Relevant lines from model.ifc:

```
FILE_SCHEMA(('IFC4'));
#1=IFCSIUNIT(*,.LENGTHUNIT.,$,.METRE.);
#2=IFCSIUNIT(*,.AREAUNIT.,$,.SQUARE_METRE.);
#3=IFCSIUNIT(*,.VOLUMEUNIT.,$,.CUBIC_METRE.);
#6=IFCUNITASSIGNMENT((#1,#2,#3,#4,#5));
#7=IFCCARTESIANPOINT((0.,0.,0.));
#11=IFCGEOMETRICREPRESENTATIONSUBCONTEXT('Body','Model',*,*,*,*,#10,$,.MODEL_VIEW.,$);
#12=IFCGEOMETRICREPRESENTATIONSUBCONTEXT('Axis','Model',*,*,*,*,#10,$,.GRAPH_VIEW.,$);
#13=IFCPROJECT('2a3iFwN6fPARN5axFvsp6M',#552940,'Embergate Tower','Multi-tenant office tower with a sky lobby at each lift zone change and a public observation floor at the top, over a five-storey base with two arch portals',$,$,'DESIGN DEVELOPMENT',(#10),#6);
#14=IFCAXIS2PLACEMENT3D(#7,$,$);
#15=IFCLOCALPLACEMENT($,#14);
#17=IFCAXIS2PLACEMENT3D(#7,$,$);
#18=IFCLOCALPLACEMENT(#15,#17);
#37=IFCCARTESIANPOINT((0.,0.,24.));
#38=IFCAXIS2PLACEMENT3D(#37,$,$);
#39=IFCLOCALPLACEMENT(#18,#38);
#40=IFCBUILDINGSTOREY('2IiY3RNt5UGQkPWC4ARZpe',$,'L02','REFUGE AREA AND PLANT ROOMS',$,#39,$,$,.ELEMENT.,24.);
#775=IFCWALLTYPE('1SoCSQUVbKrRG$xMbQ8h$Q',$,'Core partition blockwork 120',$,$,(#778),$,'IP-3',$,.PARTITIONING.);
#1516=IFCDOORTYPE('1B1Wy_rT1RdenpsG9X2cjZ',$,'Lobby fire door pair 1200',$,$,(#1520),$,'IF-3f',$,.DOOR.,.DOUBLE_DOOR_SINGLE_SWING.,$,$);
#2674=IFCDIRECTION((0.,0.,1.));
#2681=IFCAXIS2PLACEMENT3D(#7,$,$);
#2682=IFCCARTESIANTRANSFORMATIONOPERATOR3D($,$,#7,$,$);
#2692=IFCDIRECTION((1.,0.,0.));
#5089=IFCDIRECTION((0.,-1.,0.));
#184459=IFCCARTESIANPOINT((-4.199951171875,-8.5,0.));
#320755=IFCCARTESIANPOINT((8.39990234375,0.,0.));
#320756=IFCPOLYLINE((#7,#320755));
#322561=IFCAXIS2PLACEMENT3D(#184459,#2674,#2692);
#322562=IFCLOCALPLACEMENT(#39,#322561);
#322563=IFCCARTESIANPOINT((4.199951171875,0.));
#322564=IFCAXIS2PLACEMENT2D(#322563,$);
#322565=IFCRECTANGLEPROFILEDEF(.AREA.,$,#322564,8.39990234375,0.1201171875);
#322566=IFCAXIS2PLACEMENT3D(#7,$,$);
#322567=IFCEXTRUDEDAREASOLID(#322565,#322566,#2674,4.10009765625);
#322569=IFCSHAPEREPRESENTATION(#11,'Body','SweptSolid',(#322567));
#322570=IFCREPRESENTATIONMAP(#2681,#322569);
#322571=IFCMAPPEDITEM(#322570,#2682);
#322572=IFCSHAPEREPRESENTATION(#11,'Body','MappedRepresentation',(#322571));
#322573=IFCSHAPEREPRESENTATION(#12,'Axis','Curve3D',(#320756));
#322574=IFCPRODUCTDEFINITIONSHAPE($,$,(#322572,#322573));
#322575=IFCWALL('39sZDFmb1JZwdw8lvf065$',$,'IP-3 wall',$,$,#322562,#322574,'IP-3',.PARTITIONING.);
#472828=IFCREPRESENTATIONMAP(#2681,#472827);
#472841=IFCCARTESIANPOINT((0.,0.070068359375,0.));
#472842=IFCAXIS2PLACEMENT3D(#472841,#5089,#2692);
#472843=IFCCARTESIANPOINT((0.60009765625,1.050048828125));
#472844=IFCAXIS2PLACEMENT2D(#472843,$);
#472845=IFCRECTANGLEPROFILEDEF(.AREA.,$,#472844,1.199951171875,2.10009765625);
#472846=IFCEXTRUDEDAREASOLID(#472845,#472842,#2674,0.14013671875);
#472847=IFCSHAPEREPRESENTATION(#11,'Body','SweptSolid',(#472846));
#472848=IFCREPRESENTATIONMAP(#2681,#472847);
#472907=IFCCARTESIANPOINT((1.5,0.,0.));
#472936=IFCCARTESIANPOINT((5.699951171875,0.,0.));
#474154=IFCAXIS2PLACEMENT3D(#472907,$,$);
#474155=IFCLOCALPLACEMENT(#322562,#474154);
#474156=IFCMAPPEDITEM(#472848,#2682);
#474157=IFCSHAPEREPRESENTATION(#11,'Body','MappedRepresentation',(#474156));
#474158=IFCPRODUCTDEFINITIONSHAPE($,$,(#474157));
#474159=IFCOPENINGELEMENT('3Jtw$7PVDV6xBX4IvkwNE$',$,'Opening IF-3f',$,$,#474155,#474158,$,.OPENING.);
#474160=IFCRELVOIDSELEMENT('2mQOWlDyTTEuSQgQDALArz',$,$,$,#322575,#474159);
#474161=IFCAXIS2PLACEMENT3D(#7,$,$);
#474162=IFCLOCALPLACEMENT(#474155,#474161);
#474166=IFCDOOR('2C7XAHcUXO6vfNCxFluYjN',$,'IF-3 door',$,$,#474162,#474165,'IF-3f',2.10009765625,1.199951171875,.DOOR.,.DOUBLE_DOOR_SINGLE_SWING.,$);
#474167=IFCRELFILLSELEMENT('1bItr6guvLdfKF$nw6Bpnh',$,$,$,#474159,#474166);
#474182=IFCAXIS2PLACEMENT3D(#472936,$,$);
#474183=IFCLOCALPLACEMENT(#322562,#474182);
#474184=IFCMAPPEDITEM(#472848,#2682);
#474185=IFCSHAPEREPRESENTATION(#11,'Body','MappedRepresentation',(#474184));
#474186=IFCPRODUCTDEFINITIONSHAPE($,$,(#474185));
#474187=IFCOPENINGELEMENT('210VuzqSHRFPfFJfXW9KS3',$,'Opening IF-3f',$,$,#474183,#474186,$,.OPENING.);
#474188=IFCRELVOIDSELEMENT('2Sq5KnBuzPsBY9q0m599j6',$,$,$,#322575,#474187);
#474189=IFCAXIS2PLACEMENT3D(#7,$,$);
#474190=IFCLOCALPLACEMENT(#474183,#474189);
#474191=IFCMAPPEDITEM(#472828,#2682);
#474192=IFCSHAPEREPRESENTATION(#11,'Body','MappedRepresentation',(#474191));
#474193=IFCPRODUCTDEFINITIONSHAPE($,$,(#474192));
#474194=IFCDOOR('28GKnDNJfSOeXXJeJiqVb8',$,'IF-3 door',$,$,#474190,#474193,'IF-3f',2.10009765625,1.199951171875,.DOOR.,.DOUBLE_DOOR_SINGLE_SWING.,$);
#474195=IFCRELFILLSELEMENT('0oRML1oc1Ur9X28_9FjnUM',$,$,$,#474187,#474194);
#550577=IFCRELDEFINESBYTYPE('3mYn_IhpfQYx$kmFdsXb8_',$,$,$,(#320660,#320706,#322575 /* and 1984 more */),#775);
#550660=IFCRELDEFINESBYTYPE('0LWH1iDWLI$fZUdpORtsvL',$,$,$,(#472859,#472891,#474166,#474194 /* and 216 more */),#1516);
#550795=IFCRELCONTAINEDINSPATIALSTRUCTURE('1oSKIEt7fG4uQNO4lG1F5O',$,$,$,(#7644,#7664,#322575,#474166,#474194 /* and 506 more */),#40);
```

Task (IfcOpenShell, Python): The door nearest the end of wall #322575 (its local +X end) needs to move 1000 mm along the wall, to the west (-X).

```python
import ifcopenshell
import ifcopenshell.api.geometry
import ifcopenshell.util.placement
import ifcopenshell.util.unit

model = ifcopenshell.open("model.ifc")
unit_scale = ifcopenshell.util.unit.calculate_unit_scale(model)

door = model.by_guid("28GKnDNJfSOeXXJeJiqVb8")
opening = door.FillsVoids[0].RelatingOpeningElement
wall = opening.VoidsElements[0].RelatingBuildingElement

wall_matrix = ifcopenshell.util.placement.get_local_placement(wall.ObjectPlacement)
shift = wall_matrix[:3, 0] * -1 / unit_scale
before = ifcopenshell.util.placement.get_local_placement(door.ObjectPlacement)[:3, 3].copy()

# The door is placed relative to its opening, so it follows when the opening moves.
matrix = ifcopenshell.util.placement.get_local_placement(opening.ObjectPlacement)
matrix[:3, 3] += shift
ifcopenshell.api.geometry.edit_object_placement(
    model, product=opening, matrix=matrix, is_si=False, should_transform_children=True
)

after = ifcopenshell.util.placement.get_local_placement(door.ObjectPlacement)[:3, 3]
print("door moved by", (after - before).round(3) + 0.0)

model.write("model_rev.ifc")
```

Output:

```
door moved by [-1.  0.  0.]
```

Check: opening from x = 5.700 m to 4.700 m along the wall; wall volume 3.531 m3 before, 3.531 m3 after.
